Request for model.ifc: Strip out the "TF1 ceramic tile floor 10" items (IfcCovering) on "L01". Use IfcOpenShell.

First a look at what the model holds.

```python
import ifcopenshell
import ifcopenshell.util.element

model = ifcopenshell.open("model.ifc")
print(model.schema)
storey = next(s for s in model.by_type("IfcBuildingStorey") if s.Name == "L01")
coverings = [e for e in ifcopenshell.util.element.get_decomposition(storey) if e.is_a("IfcCovering")]
seen = {}
for e in coverings:
    element_type = ifcopenshell.util.element.get_type(e)
    name = element_type.Name if element_type not in (None, e) else None
    seen[name] = seen.get(name, 0) + 1
for name, count in sorted(seen.items(), key=str):
    print(count, "x", name)
```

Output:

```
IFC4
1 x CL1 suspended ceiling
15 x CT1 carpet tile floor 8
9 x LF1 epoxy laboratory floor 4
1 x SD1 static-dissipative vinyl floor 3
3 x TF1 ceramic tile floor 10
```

```python
import ifcopenshell
import ifcopenshell.api.root
import ifcopenshell.util.element

model = ifcopenshell.open("model.ifc")

storey = next(s for s in model.by_type("IfcBuildingStorey") if s.Name == "L01")
coverings = [e for e in ifcopenshell.util.element.get_decomposition(storey) if e.is_a("IfcCovering")]
targets = [e for e in coverings if (t := ifcopenshell.util.element.get_type(e)) not in (None, e) and t.Name == "TF1 ceramic tile floor 10"]

for e in targets:
    ifcopenshell.api.root.remove_product(model, product=e)
print(len(targets), "removed")

model.write("model_rev.ifc")
```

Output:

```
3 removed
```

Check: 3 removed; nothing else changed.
